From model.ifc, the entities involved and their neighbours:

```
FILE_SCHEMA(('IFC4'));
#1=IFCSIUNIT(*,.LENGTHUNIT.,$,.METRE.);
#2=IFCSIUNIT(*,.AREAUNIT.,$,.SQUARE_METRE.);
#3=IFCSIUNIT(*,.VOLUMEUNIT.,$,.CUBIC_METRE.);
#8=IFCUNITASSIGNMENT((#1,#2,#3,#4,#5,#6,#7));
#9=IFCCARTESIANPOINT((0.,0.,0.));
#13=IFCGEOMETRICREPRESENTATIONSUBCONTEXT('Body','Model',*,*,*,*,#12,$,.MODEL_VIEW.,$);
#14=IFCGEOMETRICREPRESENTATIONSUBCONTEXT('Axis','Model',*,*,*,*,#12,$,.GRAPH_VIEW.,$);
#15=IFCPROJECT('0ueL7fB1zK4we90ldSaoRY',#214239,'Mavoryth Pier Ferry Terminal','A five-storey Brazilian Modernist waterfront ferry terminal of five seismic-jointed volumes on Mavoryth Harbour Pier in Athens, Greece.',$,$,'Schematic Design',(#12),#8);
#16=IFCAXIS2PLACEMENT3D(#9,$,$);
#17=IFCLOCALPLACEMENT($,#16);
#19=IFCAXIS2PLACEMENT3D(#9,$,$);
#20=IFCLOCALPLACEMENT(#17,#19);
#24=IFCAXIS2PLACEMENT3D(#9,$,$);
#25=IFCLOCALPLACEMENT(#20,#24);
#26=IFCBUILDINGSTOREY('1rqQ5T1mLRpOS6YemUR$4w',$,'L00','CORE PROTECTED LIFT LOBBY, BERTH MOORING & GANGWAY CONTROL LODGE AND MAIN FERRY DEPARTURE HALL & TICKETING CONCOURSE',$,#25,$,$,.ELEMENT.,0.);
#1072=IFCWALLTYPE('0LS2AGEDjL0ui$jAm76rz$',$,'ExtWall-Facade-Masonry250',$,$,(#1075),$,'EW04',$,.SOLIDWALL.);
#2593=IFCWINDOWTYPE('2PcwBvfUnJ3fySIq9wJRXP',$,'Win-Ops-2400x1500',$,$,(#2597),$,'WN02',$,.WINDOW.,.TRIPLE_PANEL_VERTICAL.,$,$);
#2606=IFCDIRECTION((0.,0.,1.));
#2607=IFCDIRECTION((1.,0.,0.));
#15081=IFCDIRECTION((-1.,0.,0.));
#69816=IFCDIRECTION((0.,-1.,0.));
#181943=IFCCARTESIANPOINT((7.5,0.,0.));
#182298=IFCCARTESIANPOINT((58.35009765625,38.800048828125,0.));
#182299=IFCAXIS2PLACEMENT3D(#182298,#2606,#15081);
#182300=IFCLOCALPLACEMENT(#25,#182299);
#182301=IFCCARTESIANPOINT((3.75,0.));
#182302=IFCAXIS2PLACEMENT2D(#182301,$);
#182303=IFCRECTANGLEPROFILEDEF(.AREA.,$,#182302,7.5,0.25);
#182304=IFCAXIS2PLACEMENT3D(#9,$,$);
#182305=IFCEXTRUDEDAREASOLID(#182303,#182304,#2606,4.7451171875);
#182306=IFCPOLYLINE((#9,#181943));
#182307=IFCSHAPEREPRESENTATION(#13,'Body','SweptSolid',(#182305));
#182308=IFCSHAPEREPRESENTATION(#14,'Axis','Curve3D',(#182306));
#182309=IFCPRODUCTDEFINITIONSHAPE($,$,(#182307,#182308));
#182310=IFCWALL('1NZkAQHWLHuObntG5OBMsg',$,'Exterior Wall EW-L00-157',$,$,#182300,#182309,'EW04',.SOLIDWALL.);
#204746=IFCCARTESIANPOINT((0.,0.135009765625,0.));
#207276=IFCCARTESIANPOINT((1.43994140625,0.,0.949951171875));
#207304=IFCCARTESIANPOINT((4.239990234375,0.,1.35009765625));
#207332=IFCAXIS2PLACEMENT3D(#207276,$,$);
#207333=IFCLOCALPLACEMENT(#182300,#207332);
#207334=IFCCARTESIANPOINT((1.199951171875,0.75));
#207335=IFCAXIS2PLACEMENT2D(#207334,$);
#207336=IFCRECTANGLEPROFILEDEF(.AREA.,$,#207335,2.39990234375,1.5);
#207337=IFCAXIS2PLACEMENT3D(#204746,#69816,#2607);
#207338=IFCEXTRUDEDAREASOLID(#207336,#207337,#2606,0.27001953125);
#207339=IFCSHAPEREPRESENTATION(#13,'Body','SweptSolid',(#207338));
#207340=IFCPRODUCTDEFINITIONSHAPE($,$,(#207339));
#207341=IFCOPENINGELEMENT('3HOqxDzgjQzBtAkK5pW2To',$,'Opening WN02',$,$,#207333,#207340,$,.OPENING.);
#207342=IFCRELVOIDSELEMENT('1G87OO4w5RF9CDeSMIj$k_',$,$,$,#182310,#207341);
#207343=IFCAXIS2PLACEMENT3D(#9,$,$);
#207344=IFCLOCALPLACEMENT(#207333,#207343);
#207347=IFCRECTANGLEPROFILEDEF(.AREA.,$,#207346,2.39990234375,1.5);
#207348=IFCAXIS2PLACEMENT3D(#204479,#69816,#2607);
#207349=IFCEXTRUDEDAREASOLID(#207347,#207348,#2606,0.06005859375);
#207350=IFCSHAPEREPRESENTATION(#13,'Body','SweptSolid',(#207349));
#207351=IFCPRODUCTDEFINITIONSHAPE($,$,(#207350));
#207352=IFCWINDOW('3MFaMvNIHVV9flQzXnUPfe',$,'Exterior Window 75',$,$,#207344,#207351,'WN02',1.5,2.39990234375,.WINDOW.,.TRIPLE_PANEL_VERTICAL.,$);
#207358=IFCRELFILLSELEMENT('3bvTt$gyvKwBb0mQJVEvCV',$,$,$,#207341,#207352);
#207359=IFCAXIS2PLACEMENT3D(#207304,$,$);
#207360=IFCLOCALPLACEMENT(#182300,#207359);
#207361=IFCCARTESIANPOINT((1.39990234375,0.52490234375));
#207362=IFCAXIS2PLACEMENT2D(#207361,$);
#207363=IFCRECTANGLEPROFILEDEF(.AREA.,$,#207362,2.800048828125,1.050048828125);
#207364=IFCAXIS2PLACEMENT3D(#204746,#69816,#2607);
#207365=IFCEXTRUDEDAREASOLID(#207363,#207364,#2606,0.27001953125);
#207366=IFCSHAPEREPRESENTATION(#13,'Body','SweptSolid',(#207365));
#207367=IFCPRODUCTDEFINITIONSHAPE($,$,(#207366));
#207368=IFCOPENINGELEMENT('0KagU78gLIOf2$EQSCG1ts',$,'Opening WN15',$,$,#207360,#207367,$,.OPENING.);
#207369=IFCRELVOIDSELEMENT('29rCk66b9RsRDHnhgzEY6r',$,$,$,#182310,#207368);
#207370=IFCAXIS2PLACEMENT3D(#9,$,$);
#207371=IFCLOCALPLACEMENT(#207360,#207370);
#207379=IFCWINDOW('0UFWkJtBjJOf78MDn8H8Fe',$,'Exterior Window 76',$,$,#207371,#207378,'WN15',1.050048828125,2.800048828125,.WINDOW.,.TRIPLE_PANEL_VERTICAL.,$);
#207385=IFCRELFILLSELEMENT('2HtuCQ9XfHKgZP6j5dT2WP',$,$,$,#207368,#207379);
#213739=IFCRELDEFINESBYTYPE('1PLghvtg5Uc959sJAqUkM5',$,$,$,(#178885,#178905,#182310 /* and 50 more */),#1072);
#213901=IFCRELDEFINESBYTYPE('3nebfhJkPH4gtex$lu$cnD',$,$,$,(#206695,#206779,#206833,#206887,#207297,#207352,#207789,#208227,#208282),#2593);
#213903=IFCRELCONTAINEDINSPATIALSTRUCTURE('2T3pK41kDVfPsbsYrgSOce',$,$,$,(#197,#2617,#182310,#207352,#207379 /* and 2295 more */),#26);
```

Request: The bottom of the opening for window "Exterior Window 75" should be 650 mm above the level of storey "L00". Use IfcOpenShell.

```python
import numpy as np
import ifcopenshell
import ifcopenshell.api.geometry
import ifcopenshell.geom
import ifcopenshell.util.element
import ifcopenshell.util.placement
import ifcopenshell.util.shape
import ifcopenshell.util.unit

model = ifcopenshell.open("model.ifc")
unit_scale = ifcopenshell.util.unit.calculate_unit_scale(model)

window = model.by_guid("3MFaMvNIHVV9flQzXnUPfe")
opening = window.FillsVoids[0].RelatingOpeningElement
storey = ifcopenshell.util.element.get_container(window, ifc_class="IfcBuildingStorey")
level = ifcopenshell.util.placement.get_local_placement(storey.ObjectPlacement)[2, 3]

# The opening's origin need not be at the sill, so measure its lowest point.
shape = ifcopenshell.geom.create_shape(ifcopenshell.geom.settings(), opening)
bottom = ifcopenshell.util.shape.get_shape_bottom_elevation(shape, shape.geometry) / unit_scale
dz = level + 0.65 / unit_scale - bottom

shift = np.array([0.0, 0.0, dz])
# The window is placed relative to its opening, so it follows when the opening moves.
matrix = ifcopenshell.util.placement.get_local_placement(opening.ObjectPlacement)
matrix[:3, 3] += shift
ifcopenshell.api.geometry.edit_object_placement(
    model, product=opening, matrix=matrix, is_si=False, should_transform_children=True
)

print(f"moved by {dz * unit_scale:+.3f} m")

model.write("model_rev.ifc")
```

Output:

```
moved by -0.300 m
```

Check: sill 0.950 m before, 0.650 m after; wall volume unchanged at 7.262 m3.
